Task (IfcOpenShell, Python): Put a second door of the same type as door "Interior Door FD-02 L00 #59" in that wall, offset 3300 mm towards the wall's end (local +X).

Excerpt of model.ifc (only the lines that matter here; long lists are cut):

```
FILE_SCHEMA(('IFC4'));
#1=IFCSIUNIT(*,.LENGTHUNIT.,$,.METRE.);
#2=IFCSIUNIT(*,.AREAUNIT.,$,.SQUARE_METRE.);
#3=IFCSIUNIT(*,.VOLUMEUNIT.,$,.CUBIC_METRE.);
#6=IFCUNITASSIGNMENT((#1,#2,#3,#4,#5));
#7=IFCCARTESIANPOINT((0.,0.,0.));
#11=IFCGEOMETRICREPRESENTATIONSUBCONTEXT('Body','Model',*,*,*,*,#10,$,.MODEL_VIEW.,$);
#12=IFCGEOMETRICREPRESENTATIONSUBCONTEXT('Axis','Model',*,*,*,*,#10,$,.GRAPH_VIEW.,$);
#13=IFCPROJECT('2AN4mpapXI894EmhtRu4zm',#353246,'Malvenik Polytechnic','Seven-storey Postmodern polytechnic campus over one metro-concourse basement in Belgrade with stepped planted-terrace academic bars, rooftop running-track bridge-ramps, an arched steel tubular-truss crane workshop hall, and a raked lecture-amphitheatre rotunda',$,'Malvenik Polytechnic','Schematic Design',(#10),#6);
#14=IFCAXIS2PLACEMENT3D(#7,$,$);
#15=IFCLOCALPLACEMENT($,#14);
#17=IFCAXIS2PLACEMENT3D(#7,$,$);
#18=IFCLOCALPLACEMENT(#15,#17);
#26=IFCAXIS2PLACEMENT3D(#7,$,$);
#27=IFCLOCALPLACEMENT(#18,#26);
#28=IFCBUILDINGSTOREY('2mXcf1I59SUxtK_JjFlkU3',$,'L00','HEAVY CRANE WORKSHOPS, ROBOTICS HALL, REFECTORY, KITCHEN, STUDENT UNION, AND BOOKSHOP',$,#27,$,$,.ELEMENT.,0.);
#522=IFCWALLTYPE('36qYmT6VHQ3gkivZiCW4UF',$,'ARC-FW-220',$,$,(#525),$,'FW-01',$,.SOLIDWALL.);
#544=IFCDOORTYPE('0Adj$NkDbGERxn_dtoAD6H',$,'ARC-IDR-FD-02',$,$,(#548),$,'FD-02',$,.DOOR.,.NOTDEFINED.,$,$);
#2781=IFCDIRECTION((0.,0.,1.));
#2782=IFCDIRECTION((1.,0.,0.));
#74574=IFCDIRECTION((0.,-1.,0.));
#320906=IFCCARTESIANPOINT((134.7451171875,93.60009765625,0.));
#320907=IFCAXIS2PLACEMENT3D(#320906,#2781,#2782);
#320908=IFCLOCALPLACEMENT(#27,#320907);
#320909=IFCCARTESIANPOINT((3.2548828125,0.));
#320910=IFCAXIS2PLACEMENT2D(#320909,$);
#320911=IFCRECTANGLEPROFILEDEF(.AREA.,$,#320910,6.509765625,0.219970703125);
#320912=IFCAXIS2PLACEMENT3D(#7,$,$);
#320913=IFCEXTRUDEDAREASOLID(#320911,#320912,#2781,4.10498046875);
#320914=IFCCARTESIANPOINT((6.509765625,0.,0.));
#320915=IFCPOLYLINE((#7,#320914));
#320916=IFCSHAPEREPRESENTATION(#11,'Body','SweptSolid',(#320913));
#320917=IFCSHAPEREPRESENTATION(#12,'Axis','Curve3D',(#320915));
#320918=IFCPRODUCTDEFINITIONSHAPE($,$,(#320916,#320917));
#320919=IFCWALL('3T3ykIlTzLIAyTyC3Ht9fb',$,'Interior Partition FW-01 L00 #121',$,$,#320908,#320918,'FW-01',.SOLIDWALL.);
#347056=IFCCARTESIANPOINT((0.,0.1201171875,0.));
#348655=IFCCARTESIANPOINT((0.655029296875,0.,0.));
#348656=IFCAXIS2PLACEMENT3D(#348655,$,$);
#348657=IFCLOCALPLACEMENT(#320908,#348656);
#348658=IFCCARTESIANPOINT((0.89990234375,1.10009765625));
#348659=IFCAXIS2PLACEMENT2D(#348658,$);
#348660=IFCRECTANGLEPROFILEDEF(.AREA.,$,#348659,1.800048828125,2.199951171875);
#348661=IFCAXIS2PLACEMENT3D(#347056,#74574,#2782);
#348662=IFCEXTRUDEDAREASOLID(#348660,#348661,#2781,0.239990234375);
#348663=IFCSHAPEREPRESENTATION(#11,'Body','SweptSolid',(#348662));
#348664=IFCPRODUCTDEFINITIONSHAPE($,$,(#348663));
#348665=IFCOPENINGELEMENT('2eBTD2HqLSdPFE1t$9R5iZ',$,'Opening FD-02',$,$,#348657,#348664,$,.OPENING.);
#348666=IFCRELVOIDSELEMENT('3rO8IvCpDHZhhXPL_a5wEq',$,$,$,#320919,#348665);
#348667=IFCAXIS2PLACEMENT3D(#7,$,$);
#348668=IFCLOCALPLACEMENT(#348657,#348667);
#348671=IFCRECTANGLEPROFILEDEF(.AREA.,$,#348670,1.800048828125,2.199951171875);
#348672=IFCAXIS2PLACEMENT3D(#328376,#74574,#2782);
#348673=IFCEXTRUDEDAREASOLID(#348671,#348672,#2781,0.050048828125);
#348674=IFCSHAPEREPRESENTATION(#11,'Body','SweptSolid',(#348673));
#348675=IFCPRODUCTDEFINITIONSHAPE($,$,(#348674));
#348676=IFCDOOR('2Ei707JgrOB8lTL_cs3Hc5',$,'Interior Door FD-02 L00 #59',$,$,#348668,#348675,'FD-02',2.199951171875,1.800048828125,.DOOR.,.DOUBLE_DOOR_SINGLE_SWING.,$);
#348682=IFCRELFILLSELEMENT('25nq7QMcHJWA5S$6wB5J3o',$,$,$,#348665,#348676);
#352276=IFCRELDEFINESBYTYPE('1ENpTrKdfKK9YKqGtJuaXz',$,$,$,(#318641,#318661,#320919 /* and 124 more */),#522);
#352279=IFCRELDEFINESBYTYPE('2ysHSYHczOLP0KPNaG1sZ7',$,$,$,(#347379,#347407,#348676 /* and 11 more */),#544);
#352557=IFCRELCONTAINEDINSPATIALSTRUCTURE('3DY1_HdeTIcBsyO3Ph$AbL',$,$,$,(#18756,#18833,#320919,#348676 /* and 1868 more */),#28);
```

```python
import ifcopenshell
import ifcopenshell.api.feature
import ifcopenshell.api.geometry
import ifcopenshell.api.root
import ifcopenshell.geom
import ifcopenshell.util.element
import ifcopenshell.util.placement
import ifcopenshell.util.shape
import ifcopenshell.util.unit

model = ifcopenshell.open("model.ifc")
unit_scale = ifcopenshell.util.unit.calculate_unit_scale(model)
settings = ifcopenshell.geom.settings()


def volume(element):
    """Net volume in cubic metres, openings subtracted."""
    shape = ifcopenshell.geom.create_shape(settings, element)
    return ifcopenshell.util.shape.get_volume(shape.geometry)


door = model.by_guid("2Ei707JgrOB8lTL_cs3Hc5")
opening = door.FillsVoids[0].RelatingOpeningElement
wall = opening.VoidsElements[0].RelatingBuildingElement
before = volume(wall)
shift = ifcopenshell.util.placement.get_local_placement(wall.ObjectPlacement)[:3, 0] * 3.3 / unit_scale

# copy_class copies the void relationship, type, container and properties, but no geometry.
new_opening = ifcopenshell.api.root.copy_class(model, product=opening)
new_opening.Representation = ifcopenshell.util.element.copy_deep(
    model, opening.Representation, exclude=["IfcGeometricRepresentationContext", "IfcRepresentationMap"]
)
new_door = ifcopenshell.api.root.copy_class(model, product=door)
new_door.Representation = ifcopenshell.util.element.copy_deep(
    model, door.Representation, exclude=["IfcGeometricRepresentationContext", "IfcRepresentationMap"]
)
new_door.Tag = None
ifcopenshell.api.feature.add_filling(model, opening=new_opening, element=new_door)

for old, new in ((opening, new_opening), (door, new_door)):
    matrix = ifcopenshell.util.placement.get_local_placement(old.ObjectPlacement)
    matrix[:3, 3] += shift
    ifcopenshell.api.geometry.edit_object_placement(model, product=new, matrix=matrix, is_si=False)

after = volume(wall)

print(f"wall volume {before:.3f} -> {after:.3f} m3")

model.write("model_rev.ifc")
```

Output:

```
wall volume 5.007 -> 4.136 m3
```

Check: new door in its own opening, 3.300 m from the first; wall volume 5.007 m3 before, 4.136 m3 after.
